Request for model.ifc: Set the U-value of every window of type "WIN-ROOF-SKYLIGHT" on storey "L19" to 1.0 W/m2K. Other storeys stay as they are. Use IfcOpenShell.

First a look at what the model holds.

```python
import ifcopenshell
import ifcopenshell.util.element

model = ifcopenshell.open("model.ifc")
print(model.schema)
storey = next(s for s in model.by_type("IfcBuildingStorey") if s.Name == "L19")
windows = [e for e in ifcopenshell.util.element.get_decomposition(storey) if e.is_a("IfcWindow")]
seen = {}
for e in windows:
    element_type = ifcopenshell.util.element.get_type(e)
    key = (element_type.Name if element_type != e and element_type else None, ifcopenshell.util.element.get_pset(e, "Pset_WindowCommon", "ThermalTransmittance"))
    seen[key] = seen.get(key, 0) + 1
for (name, value), count in sorted(seen.items(), key=str):
    print(count, "x", name, "|", value)
```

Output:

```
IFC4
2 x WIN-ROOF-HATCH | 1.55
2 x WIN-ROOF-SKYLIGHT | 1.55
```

```python
import ifcopenshell
import ifcopenshell.api.pset
import ifcopenshell.util.element

model = ifcopenshell.open("model.ifc")

storey = next(s for s in model.by_type("IfcBuildingStorey") if s.Name == "L19")
windows = [e for e in ifcopenshell.util.element.get_decomposition(storey) if e.is_a("IfcWindow")]

count = 0
for e in windows:
    element_type = ifcopenshell.util.element.get_type(e)
    if element_type in (None, e) or element_type.Name != "WIN-ROOF-SKYLIGHT":
        continue
    found = ifcopenshell.util.element.get_pset(e, "Pset_WindowCommon", should_inherit=False)
    if found:
        pset = model.by_id(found["id"])
        if len(ifcopenshell.util.element.get_elements_by_pset(pset)) > 1:
            pset = ifcopenshell.api.pset.unshare_pset(model, products=[e], pset=pset)[0]
    else:
        pset = ifcopenshell.api.pset.add_pset(model, product=e, name="Pset_WindowCommon")
    ifcopenshell.api.pset.edit_pset(model, pset=pset, properties={"ThermalTransmittance": 1.0})
    count += 1

print(count, "windows updated")

model.write("model_v2.ifc")
```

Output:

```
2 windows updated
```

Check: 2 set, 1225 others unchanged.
